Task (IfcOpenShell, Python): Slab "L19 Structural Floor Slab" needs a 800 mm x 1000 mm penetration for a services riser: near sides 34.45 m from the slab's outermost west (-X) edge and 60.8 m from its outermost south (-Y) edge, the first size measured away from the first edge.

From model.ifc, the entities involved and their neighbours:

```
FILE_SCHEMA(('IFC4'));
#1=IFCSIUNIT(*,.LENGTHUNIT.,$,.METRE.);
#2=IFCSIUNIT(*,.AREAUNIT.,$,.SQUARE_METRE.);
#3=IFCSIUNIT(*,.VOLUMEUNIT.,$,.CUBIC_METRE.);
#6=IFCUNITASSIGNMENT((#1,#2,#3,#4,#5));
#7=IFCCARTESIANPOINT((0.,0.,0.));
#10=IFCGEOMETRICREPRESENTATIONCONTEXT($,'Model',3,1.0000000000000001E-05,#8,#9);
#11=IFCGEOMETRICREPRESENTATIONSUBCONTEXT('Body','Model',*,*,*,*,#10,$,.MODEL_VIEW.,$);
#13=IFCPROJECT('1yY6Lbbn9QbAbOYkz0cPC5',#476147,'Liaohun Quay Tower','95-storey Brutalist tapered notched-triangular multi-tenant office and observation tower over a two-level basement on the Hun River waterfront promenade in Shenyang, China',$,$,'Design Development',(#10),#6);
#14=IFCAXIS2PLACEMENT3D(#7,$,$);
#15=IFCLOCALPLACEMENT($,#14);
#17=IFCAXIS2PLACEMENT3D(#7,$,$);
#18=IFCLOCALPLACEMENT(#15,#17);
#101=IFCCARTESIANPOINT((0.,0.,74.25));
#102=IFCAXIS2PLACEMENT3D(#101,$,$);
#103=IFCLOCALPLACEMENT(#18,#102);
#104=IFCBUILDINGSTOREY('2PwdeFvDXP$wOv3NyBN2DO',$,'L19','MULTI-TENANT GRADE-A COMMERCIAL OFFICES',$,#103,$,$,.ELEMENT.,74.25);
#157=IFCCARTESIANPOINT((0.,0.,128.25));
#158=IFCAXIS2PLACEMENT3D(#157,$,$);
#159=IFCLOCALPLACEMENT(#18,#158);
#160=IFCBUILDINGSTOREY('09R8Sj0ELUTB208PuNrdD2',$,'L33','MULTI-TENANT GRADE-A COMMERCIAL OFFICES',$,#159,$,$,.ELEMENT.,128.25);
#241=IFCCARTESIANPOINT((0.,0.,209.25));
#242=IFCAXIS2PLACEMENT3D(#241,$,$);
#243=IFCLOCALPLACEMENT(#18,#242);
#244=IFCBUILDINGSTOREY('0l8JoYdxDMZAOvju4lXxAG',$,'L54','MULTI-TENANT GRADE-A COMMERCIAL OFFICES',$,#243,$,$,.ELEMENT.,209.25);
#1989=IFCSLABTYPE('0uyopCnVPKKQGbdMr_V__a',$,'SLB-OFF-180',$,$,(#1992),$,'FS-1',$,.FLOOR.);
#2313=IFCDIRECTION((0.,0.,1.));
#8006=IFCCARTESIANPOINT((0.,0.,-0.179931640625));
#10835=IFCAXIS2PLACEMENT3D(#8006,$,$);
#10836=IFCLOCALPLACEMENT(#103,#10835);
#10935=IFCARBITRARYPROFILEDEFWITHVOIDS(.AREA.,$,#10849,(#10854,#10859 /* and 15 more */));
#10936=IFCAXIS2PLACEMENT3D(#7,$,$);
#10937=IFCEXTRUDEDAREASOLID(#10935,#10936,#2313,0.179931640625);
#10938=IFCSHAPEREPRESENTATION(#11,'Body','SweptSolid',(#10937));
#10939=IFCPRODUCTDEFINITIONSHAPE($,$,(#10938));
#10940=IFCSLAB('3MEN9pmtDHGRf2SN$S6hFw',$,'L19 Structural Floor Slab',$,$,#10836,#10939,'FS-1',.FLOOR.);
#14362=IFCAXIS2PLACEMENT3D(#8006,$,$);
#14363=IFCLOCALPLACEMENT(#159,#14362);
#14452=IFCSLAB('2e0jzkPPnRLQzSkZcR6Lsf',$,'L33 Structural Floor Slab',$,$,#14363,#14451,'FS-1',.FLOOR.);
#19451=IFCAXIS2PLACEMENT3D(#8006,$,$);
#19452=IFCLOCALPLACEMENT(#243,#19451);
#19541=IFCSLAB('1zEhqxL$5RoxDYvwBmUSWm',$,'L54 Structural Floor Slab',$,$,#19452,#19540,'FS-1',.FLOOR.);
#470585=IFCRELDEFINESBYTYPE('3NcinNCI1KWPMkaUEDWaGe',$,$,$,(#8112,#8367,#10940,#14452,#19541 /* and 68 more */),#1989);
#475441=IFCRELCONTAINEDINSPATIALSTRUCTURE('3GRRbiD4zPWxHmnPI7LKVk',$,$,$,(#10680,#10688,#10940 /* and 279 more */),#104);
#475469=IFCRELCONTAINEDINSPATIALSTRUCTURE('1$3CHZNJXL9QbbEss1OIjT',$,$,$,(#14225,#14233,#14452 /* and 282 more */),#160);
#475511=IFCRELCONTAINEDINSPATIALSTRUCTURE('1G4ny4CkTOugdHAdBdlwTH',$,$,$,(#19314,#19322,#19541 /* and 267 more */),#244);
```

```python
import numpy as np
import ifcopenshell
import ifcopenshell.api.feature
import ifcopenshell.api.geometry
import ifcopenshell.api.root
import ifcopenshell.geom
import ifcopenshell.util.placement
import ifcopenshell.util.representation
import ifcopenshell.util.shape
import ifcopenshell.util.unit

model = ifcopenshell.open("model.ifc")
unit_scale = ifcopenshell.util.unit.calculate_unit_scale(model)
settings = ifcopenshell.geom.settings()


def volume(element):
    """Net volume in cubic metres, openings subtracted."""
    shape = ifcopenshell.geom.create_shape(settings, element)
    return ifcopenshell.util.shape.get_volume(shape.geometry)


slab = model.by_guid("3MEN9pmtDHGRf2SN$S6hFw")
before = volume(slab)

# Extent in the slab's own axes, in metres. The edges named are its -X and -Y sides.
slab_shape = ifcopenshell.geom.create_shape(settings, slab)
vertices = ifcopenshell.util.shape.get_vertices(slab_shape.geometry)
x_min, y_min, bottom = vertices.min(axis=0)
top = vertices[:, 2].max()

opening = ifcopenshell.api.root.create_entity(model, ifc_class="IfcOpeningElement", name="Services riser opening", predefined_type="OPENING")
context = ifcopenshell.util.representation.get_context(model, "Model", "Body", "MODEL_VIEW")
width, depth = 0.8, 1
outline = [(0.0, 0.0), (width, 0.0), (width, depth), (0.0, depth), (0.0, 0.0)]
# Overshoot both faces by 50 mm so the cut is clean.
shape = ifcopenshell.api.geometry.add_slab_representation(
    model, context=context, depth=top - bottom + 0.1, polyline=outline
)
ifcopenshell.api.geometry.assign_representation(model, product=opening, representation=shape)

matrix = ifcopenshell.util.placement.get_local_placement(slab.ObjectPlacement)
matrix[:, 3] = matrix @ np.append(np.array([x_min + 34.45, y_min + 60.8, bottom - 0.05]) / unit_scale, 1.0)
ifcopenshell.api.geometry.edit_object_placement(model, product=opening, matrix=matrix, is_si=False)
ifcopenshell.api.feature.add_feature(model, feature=opening, element=slab)

after = volume(slab)

print(f"slab volume {before:.3f} -> {after:.3f} m3")

model.write("model_updated.ifc")
```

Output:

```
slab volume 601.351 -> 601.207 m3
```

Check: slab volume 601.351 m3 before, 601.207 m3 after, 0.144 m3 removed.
